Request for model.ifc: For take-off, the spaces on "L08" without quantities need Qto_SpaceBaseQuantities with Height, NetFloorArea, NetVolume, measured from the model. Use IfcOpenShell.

First a look at what the model holds.

```python
import ifcopenshell
import ifcopenshell.util.element
import ifcopenshell.util.unit

model = ifcopenshell.open("model.ifc")
print(model.schema)
for unit_type in ("LENGTHUNIT", "AREAUNIT", "VOLUMEUNIT"):
    print(unit_type, ifcopenshell.util.unit.calculate_unit_scale(model, unit_type))
storey = next(s for s in model.by_type("IfcBuildingStorey") if s.Name == "L08")
spaces = [e for e in ifcopenshell.util.element.get_decomposition(storey) if e.is_a("IfcSpace")]
for e in sorted(spaces, key=lambda e: e.id()):
    print(e.id(), e.is_a(), e.Name, list(ifcopenshell.util.element.get_psets(e, qtos_only=True)), sep=" | ")
```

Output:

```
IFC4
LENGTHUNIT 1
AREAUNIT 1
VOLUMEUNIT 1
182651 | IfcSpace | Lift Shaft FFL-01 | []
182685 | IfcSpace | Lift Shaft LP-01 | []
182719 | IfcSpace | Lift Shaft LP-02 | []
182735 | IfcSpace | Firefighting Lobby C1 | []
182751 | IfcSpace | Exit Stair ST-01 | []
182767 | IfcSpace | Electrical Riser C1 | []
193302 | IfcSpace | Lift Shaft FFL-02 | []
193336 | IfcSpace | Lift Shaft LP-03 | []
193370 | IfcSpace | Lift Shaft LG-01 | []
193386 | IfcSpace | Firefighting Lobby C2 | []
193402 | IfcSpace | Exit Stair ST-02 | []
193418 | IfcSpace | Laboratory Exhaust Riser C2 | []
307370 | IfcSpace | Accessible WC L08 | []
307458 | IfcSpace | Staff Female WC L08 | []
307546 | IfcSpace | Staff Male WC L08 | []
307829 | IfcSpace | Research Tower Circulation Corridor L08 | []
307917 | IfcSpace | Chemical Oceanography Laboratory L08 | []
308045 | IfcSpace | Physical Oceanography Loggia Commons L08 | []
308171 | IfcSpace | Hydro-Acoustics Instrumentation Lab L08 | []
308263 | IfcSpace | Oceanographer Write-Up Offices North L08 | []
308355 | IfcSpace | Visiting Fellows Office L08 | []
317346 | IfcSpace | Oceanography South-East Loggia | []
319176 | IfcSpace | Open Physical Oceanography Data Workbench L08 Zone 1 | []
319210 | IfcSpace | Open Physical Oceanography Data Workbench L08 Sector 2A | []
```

```python
import ifcopenshell
import ifcopenshell.api.pset
import ifcopenshell.geom
import ifcopenshell.util.element
import ifcopenshell.util.shape
import ifcopenshell.util.unit

model = ifcopenshell.open("model.ifc")
unit_scale = ifcopenshell.util.unit.calculate_unit_scale(model)
area_scale = ifcopenshell.util.unit.calculate_unit_scale(model, "AREAUNIT")
volume_scale = ifcopenshell.util.unit.calculate_unit_scale(model, "VOLUMEUNIT")
settings = ifcopenshell.geom.settings()

storey = next(s for s in model.by_type("IfcBuildingStorey") if s.Name == "L08")
spaces = [e for e in ifcopenshell.util.element.get_decomposition(storey) if e.is_a("IfcSpace")]

for e in sorted(spaces, key=lambda e: e.id()):
    if ifcopenshell.util.element.get_psets(e, qtos_only=True, should_inherit=False):
        continue
    # Geometry comes back in metres, in the element's own axes.
    shape = ifcopenshell.geom.create_shape(settings, e)
    values = {
        "Height": ifcopenshell.util.shape.get_z(shape.geometry) / unit_scale,
        "NetFloorArea": ifcopenshell.util.shape.get_footprint_area(shape.geometry) / area_scale,
        "NetVolume": ifcopenshell.util.shape.get_volume(shape.geometry) / volume_scale,
    }
    qto = ifcopenshell.api.pset.add_qto(model, product=e, name="Qto_SpaceBaseQuantities")
    ifcopenshell.api.pset.edit_qto(model, qto=qto, properties=values)
    print(e.id(), {k: round(v, 3) for k, v in values.items()})

model.write("model-out.ifc")
```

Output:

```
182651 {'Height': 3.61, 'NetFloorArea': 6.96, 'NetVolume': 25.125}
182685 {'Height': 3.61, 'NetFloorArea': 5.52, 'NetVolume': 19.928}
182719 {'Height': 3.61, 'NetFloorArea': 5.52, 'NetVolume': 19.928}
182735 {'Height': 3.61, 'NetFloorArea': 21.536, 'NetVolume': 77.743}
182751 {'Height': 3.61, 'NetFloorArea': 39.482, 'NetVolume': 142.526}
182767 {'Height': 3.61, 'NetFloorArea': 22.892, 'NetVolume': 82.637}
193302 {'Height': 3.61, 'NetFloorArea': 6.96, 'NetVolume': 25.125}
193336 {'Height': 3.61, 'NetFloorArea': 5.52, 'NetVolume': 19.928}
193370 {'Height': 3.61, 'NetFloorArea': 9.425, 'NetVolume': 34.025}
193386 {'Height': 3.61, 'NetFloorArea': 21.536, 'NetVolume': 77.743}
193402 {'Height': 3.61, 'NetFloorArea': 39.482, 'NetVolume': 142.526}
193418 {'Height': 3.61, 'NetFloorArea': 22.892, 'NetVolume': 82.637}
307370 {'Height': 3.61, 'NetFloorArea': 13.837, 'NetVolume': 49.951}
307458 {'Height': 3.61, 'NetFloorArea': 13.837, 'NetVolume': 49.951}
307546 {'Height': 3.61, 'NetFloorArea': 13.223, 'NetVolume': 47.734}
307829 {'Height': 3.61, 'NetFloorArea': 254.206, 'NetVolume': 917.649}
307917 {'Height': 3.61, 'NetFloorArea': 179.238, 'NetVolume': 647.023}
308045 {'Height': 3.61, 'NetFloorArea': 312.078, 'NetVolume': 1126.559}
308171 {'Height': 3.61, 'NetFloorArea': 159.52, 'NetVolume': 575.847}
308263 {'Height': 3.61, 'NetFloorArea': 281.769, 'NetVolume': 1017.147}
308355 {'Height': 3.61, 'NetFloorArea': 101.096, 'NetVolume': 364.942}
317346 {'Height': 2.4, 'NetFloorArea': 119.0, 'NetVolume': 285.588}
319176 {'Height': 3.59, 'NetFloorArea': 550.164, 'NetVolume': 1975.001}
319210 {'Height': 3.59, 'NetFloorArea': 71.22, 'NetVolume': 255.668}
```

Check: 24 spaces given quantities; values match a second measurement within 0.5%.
